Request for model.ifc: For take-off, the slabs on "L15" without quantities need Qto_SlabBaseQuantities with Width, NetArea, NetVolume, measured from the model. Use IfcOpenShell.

First a look at what the model holds.

```python
import ifcopenshell
import ifcopenshell.util.element
import ifcopenshell.util.unit

model = ifcopenshell.open("model.ifc")
print(model.schema)
for unit_type in ("LENGTHUNIT", "AREAUNIT", "VOLUMEUNIT"):
    print(unit_type, ifcopenshell.util.unit.calculate_unit_scale(model, unit_type))
storey = next(s for s in model.by_type("IfcBuildingStorey") if s.Name == "L15")
slabs = [e for e in ifcopenshell.util.element.get_decomposition(storey) if e.is_a("IfcSlab")]
for e in sorted(slabs, key=lambda e: e.id()):
    print(e.id(), e.is_a(), e.Name, list(ifcopenshell.util.element.get_psets(e, qtos_only=True)), sep=" | ")
```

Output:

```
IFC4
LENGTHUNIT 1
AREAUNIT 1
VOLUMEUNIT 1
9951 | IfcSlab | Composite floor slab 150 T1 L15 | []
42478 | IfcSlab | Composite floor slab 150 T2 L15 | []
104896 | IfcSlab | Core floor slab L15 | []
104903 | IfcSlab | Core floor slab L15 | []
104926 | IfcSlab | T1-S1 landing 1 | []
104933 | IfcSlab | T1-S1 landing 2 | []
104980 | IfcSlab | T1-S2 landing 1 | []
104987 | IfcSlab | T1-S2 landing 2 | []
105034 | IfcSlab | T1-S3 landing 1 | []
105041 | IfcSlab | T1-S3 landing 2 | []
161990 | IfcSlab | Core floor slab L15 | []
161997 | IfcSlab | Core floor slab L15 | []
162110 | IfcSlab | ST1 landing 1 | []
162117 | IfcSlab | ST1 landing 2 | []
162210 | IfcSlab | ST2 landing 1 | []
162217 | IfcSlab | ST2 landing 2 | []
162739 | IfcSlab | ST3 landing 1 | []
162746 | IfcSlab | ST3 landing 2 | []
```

```python
import ifcopenshell
import ifcopenshell.api.pset
import ifcopenshell.geom
import ifcopenshell.util.element
import ifcopenshell.util.shape
import ifcopenshell.util.unit

model = ifcopenshell.open("model.ifc")
unit_scale = ifcopenshell.util.unit.calculate_unit_scale(model)
area_scale = ifcopenshell.util.unit.calculate_unit_scale(model, "AREAUNIT")
volume_scale = ifcopenshell.util.unit.calculate_unit_scale(model, "VOLUMEUNIT")
settings = ifcopenshell.geom.settings()

storey = next(s for s in model.by_type("IfcBuildingStorey") if s.Name == "L15")
slabs = [e for e in ifcopenshell.util.element.get_decomposition(storey) if e.is_a("IfcSlab")]

for e in sorted(slabs, key=lambda e: e.id()):
    if ifcopenshell.util.element.get_psets(e, qtos_only=True, should_inherit=False):
        continue
    # Geometry comes back in metres, in the element's own axes.
    shape = ifcopenshell.geom.create_shape(settings, e)
    values = {
        "Width": ifcopenshell.util.shape.get_z(shape.geometry) / unit_scale,
        "NetArea": ifcopenshell.util.shape.get_footprint_area(shape.geometry) / area_scale,
        "NetVolume": ifcopenshell.util.shape.get_volume(shape.geometry) / volume_scale,
    }
    qto = ifcopenshell.api.pset.add_qto(model, product=e, name="Qto_SlabBaseQuantities")
    ifcopenshell.api.pset.edit_qto(model, qto=qto, properties=values)
    print(e.id(), {k: round(v, 3) for k, v in values.items()})

model.write("model_edited.ifc")
```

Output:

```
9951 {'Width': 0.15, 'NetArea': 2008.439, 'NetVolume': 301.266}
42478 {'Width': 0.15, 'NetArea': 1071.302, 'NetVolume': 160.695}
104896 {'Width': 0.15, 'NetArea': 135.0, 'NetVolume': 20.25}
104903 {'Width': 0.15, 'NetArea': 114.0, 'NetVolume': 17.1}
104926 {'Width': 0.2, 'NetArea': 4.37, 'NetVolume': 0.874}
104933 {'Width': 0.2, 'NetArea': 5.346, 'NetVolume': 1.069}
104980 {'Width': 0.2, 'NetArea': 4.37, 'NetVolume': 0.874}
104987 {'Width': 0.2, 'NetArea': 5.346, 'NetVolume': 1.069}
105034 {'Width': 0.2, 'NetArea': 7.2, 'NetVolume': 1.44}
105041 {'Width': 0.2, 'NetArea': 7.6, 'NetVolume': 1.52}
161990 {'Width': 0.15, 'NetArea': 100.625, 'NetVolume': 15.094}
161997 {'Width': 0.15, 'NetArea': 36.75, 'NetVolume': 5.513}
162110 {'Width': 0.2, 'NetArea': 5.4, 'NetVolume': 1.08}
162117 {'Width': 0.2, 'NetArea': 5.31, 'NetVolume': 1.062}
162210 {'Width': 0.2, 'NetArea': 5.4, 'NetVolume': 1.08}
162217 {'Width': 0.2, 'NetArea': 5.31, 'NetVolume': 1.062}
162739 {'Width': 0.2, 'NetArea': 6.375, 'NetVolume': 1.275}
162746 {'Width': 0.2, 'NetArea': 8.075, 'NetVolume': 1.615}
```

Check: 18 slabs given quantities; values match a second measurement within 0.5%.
